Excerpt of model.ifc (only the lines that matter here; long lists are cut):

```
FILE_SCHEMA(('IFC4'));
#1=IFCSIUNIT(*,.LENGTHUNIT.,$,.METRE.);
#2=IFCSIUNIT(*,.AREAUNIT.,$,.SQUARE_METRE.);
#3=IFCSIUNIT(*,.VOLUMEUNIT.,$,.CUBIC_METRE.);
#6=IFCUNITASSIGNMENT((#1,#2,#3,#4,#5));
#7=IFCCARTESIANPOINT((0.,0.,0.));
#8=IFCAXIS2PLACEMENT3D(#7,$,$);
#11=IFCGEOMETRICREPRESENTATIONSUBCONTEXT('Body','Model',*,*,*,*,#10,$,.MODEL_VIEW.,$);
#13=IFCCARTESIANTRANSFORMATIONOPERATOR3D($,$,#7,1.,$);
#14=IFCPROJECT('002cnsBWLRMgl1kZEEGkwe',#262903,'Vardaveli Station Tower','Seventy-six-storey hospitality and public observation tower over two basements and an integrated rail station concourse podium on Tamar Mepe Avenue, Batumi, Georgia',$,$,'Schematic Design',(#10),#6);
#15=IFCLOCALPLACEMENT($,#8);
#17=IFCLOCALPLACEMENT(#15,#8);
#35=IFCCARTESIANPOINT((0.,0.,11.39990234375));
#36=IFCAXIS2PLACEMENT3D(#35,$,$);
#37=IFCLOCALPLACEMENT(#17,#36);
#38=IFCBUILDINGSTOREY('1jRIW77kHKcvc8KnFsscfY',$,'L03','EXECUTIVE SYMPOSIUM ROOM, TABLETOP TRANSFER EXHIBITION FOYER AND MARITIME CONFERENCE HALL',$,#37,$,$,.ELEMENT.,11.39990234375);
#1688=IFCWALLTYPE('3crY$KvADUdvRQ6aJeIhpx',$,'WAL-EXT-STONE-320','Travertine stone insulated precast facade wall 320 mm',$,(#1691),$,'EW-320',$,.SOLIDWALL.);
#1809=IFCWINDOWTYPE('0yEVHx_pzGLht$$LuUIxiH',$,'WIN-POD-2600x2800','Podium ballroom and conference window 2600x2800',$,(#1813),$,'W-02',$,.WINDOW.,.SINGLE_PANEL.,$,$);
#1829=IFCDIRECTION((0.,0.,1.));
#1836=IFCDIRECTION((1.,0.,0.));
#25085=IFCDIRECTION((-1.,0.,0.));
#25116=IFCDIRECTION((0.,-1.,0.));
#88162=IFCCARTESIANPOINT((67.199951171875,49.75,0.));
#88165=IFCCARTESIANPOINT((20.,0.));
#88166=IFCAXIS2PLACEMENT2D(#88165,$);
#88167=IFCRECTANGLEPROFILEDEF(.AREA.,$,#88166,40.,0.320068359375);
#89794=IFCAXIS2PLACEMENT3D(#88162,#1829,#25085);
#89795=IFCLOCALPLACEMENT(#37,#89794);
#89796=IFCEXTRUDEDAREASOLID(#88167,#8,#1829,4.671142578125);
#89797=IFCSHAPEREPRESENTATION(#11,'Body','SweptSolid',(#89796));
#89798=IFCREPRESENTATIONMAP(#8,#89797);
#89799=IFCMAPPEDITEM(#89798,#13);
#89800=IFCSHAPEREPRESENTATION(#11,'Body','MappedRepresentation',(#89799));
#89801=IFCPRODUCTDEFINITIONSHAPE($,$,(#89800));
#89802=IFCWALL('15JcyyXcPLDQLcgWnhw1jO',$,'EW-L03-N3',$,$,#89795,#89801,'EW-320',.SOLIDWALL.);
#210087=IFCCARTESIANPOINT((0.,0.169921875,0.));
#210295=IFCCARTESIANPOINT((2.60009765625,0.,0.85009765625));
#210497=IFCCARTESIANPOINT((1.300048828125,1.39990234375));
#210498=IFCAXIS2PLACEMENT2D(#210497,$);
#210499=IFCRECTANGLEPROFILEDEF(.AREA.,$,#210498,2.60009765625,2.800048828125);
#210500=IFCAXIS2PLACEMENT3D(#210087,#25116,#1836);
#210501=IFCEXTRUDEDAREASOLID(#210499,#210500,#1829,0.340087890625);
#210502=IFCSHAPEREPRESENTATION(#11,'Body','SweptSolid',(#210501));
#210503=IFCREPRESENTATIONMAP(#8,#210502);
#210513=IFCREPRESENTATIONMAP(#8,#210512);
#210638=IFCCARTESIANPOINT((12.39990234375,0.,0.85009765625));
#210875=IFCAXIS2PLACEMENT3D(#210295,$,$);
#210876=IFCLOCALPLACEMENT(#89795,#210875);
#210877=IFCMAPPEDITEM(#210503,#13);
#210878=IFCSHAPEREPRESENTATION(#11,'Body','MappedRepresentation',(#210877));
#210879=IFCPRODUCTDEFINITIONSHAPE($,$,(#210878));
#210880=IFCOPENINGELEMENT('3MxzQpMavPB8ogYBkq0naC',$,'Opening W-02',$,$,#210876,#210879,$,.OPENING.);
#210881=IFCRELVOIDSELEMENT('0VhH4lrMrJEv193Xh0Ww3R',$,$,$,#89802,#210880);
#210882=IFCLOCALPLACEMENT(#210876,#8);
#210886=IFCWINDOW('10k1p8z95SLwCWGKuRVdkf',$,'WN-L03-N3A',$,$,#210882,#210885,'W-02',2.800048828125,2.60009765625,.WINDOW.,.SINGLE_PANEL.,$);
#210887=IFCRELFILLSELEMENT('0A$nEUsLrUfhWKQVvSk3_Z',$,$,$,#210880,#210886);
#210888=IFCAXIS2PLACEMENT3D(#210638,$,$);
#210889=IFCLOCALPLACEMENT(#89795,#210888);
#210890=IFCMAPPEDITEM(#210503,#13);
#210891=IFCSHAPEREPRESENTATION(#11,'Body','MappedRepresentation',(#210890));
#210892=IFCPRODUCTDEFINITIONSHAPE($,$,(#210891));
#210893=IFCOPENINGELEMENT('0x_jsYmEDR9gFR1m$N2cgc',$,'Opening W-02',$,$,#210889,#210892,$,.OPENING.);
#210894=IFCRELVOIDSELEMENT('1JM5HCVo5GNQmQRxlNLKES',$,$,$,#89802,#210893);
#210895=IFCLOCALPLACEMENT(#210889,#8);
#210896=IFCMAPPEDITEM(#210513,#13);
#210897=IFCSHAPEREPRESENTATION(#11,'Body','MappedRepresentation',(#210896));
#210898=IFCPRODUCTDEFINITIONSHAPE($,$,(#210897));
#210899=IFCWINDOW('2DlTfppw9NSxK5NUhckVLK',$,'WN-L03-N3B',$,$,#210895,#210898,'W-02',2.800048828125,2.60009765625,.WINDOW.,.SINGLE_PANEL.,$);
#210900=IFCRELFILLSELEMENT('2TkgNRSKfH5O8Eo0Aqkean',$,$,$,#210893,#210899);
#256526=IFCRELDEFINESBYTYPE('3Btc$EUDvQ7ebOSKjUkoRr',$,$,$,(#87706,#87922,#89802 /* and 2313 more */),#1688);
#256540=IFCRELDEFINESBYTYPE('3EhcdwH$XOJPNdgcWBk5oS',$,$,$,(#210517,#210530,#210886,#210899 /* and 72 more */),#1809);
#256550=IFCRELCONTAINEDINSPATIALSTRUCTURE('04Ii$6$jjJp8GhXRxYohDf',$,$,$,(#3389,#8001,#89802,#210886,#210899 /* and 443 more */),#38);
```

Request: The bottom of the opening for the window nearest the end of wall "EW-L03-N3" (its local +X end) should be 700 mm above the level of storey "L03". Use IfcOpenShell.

```python
import numpy as np
import ifcopenshell
import ifcopenshell.api.geometry
import ifcopenshell.geom
import ifcopenshell.util.element
import ifcopenshell.util.placement
import ifcopenshell.util.shape
import ifcopenshell.util.unit

model = ifcopenshell.open("model.ifc")
unit_scale = ifcopenshell.util.unit.calculate_unit_scale(model)

window = model.by_guid("2DlTfppw9NSxK5NUhckVLK")
opening = window.FillsVoids[0].RelatingOpeningElement
storey = ifcopenshell.util.element.get_container(window, ifc_class="IfcBuildingStorey")
level = ifcopenshell.util.placement.get_local_placement(storey.ObjectPlacement)[2, 3]

# The opening's origin need not be at the sill, so measure its lowest point.
shape = ifcopenshell.geom.create_shape(ifcopenshell.geom.settings(), opening)
bottom = ifcopenshell.util.shape.get_shape_bottom_elevation(shape, shape.geometry) / unit_scale
dz = level + 0.7 / unit_scale - bottom

shift = np.array([0.0, 0.0, dz])
# The window is placed relative to its opening, so it follows when the opening moves.
matrix = ifcopenshell.util.placement.get_local_placement(opening.ObjectPlacement)
matrix[:3, 3] += shift
ifcopenshell.api.geometry.edit_object_placement(
    model, product=opening, matrix=matrix, is_si=False, should_transform_children=True
)

print(f"moved by {dz * unit_scale:+.3f} m")

model.write("model-out.ifc")
```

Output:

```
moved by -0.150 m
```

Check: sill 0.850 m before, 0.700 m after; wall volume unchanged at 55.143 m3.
